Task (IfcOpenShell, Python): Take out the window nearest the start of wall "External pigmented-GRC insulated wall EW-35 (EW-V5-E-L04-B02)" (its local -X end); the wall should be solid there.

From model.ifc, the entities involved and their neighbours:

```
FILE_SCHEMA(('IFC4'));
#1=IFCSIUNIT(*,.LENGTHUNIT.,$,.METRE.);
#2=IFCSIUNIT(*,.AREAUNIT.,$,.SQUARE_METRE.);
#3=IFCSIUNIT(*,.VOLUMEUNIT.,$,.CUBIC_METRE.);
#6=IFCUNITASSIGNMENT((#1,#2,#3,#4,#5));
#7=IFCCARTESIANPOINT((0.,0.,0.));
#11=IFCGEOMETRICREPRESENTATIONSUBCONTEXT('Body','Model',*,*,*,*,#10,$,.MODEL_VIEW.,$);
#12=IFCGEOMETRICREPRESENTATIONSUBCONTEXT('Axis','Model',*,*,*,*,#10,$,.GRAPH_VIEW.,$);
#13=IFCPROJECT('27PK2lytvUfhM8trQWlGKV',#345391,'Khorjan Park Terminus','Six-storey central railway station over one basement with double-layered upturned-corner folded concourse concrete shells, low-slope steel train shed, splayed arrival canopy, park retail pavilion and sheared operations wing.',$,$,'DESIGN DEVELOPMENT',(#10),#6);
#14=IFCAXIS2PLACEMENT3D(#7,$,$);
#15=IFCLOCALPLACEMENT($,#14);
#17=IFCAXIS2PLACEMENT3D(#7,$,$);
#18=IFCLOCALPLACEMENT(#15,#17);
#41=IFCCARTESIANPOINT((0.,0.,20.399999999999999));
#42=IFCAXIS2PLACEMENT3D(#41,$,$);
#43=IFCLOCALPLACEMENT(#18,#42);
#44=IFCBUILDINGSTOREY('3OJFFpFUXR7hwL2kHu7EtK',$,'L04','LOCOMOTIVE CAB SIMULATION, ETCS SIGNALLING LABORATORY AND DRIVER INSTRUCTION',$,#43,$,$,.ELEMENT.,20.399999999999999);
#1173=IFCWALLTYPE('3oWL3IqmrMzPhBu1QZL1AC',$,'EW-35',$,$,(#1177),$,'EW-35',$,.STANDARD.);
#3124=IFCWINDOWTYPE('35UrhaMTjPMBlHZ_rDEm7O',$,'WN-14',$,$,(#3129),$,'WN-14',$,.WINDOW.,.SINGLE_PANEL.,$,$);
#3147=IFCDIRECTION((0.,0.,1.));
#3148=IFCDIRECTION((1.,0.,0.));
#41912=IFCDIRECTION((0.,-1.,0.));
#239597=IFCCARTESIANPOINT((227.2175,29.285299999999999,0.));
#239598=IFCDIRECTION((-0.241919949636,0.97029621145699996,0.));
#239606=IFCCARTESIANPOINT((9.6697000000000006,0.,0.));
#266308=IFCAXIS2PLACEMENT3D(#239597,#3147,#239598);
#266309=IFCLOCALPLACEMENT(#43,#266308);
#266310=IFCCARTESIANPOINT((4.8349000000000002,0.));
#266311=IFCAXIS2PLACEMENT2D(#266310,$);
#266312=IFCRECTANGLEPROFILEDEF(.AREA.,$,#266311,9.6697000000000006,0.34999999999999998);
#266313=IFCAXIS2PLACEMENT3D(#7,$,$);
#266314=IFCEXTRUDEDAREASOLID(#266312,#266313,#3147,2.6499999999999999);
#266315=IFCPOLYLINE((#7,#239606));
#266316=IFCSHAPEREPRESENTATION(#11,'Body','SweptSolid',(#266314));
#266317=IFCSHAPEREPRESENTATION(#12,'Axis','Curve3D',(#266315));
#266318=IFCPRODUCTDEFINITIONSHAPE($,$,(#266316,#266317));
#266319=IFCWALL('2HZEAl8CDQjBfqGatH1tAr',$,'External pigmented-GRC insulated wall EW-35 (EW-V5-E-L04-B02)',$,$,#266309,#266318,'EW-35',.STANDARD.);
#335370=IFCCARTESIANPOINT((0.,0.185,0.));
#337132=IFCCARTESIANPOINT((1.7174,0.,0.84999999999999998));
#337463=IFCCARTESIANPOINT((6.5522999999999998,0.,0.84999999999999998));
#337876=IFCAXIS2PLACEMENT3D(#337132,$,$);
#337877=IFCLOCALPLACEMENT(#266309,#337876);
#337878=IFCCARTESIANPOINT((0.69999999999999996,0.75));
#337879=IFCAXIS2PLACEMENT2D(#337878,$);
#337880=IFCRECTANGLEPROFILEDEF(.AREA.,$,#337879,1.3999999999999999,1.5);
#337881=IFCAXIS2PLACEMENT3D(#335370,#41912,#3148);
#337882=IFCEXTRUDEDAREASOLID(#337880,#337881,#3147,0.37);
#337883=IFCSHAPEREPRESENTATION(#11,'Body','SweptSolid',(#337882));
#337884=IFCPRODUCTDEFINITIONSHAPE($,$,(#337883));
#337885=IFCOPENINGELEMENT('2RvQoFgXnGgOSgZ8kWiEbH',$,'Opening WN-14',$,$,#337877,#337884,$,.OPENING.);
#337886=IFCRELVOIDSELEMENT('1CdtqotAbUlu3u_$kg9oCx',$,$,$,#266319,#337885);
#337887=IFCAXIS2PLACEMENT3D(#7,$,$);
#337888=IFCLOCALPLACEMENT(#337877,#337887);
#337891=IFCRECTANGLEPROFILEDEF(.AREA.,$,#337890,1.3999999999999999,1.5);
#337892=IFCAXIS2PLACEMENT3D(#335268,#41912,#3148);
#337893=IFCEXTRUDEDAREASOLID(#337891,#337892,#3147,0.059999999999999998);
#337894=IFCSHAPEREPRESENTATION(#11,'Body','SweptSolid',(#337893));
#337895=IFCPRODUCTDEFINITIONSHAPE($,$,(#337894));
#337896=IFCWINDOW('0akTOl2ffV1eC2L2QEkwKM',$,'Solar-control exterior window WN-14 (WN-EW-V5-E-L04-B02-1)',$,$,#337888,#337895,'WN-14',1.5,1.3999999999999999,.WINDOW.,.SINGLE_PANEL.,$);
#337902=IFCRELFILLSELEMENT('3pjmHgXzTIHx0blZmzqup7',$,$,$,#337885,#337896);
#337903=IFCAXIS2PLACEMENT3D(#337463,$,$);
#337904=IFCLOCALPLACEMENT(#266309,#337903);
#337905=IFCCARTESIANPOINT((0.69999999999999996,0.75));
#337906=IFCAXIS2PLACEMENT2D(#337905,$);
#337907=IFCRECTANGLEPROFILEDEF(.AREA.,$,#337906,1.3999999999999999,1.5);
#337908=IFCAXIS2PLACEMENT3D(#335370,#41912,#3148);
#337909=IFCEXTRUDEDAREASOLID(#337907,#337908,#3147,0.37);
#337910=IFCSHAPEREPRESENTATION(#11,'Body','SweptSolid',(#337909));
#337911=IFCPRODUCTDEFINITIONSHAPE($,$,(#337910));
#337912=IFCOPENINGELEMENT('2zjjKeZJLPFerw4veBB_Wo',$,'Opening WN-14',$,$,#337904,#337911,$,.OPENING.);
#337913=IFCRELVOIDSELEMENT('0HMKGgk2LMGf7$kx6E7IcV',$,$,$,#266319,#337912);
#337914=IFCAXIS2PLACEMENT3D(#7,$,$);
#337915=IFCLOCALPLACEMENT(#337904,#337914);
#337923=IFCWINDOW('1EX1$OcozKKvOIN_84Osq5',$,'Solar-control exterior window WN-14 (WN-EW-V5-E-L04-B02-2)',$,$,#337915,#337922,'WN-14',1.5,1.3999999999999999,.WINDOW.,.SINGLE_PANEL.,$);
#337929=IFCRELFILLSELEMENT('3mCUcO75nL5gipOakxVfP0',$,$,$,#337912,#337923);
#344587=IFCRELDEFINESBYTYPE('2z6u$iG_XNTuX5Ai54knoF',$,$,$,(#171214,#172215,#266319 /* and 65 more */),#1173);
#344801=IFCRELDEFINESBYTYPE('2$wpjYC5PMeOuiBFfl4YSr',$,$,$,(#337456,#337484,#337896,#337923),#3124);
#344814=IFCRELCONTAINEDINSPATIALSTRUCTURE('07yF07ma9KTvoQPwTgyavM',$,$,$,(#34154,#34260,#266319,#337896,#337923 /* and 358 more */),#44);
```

```python
import ifcopenshell
import ifcopenshell.api.feature
import ifcopenshell.api.root
import ifcopenshell.geom
import ifcopenshell.util.shape

model = ifcopenshell.open("model.ifc")
settings = ifcopenshell.geom.settings()


def volume(element):
    """Net volume in cubic metres, openings subtracted."""
    shape = ifcopenshell.geom.create_shape(settings, element)
    return ifcopenshell.util.shape.get_volume(shape.geometry)


window = model.by_guid("0akTOl2ffV1eC2L2QEkwKM")
opening = window.FillsVoids[0].RelatingOpeningElement
wall = opening.VoidsElements[0].RelatingBuildingElement
before = volume(wall)

ifcopenshell.api.root.remove_product(model, product=window)
ifcopenshell.api.feature.remove_feature(model, feature=opening)

after = volume(wall)

print(f"wall volume {before:.3f} -> {after:.3f} m3")

model.write("model_v2.ifc")
```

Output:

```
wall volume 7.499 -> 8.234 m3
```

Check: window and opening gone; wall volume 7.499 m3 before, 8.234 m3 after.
